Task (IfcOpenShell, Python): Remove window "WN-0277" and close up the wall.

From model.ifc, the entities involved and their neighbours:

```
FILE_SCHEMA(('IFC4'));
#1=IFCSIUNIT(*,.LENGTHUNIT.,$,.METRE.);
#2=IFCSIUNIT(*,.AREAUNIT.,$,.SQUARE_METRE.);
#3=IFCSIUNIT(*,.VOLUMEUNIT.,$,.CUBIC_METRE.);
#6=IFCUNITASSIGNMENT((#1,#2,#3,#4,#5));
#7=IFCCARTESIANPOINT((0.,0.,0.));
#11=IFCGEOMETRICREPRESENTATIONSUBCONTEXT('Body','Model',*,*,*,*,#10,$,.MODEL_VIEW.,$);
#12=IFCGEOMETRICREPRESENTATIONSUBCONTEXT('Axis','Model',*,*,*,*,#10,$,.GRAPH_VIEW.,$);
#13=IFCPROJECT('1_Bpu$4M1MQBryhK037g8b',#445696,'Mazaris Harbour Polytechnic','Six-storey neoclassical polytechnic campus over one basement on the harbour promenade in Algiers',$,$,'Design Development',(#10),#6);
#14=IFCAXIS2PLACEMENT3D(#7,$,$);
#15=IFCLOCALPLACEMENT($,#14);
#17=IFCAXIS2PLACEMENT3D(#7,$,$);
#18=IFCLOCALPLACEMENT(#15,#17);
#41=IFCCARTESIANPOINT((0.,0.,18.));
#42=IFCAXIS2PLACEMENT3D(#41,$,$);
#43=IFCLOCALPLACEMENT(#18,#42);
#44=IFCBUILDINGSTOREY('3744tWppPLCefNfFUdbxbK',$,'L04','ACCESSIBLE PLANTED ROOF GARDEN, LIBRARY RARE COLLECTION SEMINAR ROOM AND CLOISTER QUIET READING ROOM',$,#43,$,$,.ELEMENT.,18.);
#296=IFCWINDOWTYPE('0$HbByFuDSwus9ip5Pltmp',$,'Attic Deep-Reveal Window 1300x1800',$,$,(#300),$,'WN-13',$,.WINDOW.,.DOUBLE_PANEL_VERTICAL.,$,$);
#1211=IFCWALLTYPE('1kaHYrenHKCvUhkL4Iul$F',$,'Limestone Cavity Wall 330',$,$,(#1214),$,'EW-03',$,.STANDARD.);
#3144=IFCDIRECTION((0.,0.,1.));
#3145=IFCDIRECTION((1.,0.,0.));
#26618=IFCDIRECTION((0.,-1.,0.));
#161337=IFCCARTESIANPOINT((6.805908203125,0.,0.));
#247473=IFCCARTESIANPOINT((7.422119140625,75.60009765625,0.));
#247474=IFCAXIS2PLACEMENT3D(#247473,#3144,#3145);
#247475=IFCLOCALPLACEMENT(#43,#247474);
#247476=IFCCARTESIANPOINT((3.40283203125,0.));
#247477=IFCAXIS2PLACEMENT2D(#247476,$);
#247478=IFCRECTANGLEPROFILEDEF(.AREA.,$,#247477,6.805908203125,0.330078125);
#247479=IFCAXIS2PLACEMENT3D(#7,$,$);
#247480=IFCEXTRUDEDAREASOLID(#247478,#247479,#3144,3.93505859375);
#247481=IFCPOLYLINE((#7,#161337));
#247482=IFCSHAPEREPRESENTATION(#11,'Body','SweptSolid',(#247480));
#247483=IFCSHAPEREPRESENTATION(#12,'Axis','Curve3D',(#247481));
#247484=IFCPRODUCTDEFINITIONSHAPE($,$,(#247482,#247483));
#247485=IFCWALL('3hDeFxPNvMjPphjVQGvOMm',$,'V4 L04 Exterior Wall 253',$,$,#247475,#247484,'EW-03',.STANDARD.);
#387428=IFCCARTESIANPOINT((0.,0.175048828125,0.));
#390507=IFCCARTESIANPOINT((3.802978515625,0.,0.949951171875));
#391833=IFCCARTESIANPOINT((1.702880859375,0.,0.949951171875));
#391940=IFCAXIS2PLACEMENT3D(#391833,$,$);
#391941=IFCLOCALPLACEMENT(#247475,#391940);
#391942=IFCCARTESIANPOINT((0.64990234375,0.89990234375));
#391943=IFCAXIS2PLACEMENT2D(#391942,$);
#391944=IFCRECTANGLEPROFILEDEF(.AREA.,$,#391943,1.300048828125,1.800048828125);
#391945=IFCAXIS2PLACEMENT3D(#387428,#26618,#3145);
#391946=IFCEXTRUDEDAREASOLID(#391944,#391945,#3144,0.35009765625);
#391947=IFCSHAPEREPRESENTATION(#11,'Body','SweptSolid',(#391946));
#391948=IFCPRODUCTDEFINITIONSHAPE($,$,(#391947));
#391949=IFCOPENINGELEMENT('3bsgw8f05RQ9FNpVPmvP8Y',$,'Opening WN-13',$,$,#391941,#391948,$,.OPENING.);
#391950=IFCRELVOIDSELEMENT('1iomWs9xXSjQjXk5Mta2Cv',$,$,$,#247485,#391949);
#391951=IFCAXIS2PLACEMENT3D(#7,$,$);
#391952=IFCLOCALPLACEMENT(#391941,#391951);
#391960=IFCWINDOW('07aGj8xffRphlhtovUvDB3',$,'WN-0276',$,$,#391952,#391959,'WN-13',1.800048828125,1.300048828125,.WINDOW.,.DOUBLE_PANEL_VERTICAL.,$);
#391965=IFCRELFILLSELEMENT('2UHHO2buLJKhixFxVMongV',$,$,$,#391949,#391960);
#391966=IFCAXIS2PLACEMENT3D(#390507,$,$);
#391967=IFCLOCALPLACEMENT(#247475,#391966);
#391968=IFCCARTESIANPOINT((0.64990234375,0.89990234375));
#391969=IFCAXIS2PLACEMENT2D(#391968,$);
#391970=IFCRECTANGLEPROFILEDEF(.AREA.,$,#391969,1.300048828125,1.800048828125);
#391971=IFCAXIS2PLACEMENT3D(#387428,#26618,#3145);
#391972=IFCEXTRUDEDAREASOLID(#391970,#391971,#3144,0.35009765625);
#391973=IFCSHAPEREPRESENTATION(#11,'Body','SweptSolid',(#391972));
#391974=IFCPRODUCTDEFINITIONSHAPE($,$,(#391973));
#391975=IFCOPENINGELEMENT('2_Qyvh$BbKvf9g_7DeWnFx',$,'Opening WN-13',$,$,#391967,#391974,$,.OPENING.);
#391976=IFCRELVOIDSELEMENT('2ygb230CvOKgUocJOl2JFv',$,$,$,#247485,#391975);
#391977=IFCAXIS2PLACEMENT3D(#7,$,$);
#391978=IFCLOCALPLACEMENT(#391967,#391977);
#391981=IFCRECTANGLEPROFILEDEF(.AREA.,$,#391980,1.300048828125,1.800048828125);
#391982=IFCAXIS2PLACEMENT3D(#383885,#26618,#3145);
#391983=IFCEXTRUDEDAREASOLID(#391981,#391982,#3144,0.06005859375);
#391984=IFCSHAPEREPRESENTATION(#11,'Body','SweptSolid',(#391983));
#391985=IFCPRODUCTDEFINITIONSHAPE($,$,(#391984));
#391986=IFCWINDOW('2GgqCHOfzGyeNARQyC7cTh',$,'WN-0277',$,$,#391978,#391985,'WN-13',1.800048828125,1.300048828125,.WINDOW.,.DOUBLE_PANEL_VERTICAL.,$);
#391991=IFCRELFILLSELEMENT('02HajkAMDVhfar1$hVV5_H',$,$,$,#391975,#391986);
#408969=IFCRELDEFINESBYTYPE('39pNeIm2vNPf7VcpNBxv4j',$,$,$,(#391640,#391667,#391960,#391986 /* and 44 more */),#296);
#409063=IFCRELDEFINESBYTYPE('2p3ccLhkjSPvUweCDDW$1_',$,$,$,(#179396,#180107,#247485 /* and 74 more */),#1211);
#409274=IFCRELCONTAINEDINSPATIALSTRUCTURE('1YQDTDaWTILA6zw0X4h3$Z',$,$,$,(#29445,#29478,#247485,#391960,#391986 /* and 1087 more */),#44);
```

```python
import ifcopenshell
import ifcopenshell.api.feature
import ifcopenshell.api.root
import ifcopenshell.geom
import ifcopenshell.util.shape

model = ifcopenshell.open("model.ifc")
settings = ifcopenshell.geom.settings()


def volume(element):
    """Net volume in cubic metres, openings subtracted."""
    shape = ifcopenshell.geom.create_shape(settings, element)
    return ifcopenshell.util.shape.get_volume(shape.geometry)


window = model.by_id(391986)
opening = window.FillsVoids[0].RelatingOpeningElement
wall = opening.VoidsElements[0].RelatingBuildingElement
before = volume(wall)

ifcopenshell.api.root.remove_product(model, product=window)
ifcopenshell.api.feature.remove_feature(model, feature=opening)

after = volume(wall)

print(f"wall volume {before:.3f} -> {after:.3f} m3")

model.write("model_rev.ifc")
```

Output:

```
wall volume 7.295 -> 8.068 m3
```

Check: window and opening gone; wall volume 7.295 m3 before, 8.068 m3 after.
